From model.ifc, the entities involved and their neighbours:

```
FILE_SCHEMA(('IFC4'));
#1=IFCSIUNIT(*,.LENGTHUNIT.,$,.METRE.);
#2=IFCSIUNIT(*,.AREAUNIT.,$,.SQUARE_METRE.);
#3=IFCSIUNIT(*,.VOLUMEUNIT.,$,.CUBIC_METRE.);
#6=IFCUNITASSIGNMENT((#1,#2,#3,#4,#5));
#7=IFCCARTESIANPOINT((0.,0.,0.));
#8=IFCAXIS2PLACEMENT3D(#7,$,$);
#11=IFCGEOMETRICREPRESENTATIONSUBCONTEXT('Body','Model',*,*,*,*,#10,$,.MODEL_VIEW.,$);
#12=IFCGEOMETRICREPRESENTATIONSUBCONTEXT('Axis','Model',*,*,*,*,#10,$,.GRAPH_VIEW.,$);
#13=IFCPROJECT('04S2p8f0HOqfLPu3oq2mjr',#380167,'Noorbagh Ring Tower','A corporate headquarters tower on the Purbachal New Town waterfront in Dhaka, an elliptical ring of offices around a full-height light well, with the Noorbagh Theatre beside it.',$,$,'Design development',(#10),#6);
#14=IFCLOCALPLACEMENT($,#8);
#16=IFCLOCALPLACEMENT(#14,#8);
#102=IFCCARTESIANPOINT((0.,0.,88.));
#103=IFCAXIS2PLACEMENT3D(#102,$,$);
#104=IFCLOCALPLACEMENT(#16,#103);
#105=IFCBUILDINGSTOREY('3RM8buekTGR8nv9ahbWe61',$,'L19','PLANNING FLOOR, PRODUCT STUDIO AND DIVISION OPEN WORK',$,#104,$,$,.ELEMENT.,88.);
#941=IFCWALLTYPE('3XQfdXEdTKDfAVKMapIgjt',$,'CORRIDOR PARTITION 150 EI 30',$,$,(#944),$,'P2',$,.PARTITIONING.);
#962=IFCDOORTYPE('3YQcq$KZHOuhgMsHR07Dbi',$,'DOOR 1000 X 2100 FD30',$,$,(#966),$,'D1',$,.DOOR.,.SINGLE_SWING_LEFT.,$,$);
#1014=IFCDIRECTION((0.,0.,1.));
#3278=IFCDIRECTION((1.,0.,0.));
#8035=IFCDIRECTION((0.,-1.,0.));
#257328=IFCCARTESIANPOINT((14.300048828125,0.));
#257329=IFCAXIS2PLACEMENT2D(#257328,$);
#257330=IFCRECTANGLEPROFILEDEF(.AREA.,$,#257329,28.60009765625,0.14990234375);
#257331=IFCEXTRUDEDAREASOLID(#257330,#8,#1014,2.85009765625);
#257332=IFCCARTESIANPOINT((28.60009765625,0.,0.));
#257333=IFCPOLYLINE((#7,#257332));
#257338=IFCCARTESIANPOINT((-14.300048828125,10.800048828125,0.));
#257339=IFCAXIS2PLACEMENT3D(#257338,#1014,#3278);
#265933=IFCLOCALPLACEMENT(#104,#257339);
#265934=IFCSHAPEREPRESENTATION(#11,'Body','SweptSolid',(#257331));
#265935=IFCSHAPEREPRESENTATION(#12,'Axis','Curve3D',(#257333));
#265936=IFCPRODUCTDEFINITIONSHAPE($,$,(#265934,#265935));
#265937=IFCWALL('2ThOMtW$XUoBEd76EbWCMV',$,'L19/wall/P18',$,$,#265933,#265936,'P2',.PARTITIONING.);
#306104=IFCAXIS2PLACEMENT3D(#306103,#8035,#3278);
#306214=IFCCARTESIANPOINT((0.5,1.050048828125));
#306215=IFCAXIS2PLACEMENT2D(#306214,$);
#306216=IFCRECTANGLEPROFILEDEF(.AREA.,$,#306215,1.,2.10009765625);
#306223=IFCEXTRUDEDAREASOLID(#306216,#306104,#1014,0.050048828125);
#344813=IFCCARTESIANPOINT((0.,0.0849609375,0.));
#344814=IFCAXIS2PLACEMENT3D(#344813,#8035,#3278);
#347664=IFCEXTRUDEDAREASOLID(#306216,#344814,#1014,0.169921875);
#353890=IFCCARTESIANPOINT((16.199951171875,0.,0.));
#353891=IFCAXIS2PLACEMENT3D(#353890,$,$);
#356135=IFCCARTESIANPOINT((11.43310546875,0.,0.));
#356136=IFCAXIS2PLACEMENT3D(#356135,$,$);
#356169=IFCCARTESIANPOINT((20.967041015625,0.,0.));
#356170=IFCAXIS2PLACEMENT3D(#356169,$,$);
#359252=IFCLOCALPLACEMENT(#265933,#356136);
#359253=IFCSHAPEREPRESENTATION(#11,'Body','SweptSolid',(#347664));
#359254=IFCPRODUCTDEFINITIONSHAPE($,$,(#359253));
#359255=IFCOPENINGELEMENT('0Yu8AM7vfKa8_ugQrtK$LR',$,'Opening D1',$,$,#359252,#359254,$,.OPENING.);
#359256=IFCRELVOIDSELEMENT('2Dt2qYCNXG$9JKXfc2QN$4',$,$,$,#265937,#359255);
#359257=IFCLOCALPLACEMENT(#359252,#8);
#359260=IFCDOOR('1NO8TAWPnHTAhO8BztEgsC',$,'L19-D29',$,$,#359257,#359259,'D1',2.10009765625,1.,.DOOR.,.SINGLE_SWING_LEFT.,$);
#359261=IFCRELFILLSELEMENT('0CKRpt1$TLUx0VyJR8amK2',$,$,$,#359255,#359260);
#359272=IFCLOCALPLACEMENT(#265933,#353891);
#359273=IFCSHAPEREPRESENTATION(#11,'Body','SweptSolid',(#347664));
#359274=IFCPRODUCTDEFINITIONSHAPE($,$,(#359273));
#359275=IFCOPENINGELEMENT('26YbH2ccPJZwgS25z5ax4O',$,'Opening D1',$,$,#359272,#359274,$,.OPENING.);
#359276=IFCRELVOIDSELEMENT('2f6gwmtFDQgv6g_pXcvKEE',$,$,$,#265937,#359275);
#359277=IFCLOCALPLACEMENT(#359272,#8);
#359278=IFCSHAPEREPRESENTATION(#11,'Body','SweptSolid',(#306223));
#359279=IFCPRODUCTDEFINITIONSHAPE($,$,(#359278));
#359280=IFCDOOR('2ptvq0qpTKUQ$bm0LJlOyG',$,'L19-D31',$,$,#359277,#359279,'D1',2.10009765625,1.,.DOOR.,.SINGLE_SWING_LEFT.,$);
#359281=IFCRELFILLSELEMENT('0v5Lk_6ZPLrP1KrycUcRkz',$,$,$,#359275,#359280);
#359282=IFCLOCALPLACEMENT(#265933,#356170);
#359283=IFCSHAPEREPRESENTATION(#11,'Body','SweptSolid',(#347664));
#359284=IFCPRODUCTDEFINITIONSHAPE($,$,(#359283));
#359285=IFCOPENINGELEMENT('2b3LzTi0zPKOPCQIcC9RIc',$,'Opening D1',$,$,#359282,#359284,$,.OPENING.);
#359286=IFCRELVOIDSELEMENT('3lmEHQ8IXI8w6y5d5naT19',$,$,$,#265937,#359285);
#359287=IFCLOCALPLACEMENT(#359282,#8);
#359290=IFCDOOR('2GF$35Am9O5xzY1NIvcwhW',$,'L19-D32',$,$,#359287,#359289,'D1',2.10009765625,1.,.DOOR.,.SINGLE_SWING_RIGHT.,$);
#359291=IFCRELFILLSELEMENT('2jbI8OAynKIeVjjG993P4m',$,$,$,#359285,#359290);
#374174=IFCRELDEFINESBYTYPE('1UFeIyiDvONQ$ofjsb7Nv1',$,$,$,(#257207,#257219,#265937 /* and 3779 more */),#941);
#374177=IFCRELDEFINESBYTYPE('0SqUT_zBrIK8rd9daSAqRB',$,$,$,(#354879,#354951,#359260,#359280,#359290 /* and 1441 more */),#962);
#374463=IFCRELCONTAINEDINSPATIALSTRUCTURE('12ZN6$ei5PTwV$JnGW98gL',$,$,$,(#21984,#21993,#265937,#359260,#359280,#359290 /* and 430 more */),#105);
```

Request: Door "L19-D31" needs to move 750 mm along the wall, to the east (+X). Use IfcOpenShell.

```python
import ifcopenshell
import ifcopenshell.api.geometry
import ifcopenshell.util.placement

model = ifcopenshell.open("model.ifc")

door = model.by_guid("2ptvq0qpTKUQ$bm0LJlOyG")
opening = door.FillsVoids[0].RelatingOpeningElement
wall = opening.VoidsElements[0].RelatingBuildingElement

wall_matrix = ifcopenshell.util.placement.get_local_placement(wall.ObjectPlacement)
shift = wall_matrix[:3, 0] * 0.75
before = ifcopenshell.util.placement.get_local_placement(door.ObjectPlacement)[:3, 3].copy()

# The door is placed relative to its opening, so it follows when the opening moves.
matrix = ifcopenshell.util.placement.get_local_placement(opening.ObjectPlacement)
matrix[:3, 3] += shift
ifcopenshell.api.geometry.edit_object_placement(
    model, product=opening, matrix=matrix, is_si=False, should_transform_children=True
)

after = ifcopenshell.util.placement.get_local_placement(door.ObjectPlacement)[:3, 3]
print("door moved by", (after - before).round(3) + 0.0)

model.write("model_v2.ifc")
```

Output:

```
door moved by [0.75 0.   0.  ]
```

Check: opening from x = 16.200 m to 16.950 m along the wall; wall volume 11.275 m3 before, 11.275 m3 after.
